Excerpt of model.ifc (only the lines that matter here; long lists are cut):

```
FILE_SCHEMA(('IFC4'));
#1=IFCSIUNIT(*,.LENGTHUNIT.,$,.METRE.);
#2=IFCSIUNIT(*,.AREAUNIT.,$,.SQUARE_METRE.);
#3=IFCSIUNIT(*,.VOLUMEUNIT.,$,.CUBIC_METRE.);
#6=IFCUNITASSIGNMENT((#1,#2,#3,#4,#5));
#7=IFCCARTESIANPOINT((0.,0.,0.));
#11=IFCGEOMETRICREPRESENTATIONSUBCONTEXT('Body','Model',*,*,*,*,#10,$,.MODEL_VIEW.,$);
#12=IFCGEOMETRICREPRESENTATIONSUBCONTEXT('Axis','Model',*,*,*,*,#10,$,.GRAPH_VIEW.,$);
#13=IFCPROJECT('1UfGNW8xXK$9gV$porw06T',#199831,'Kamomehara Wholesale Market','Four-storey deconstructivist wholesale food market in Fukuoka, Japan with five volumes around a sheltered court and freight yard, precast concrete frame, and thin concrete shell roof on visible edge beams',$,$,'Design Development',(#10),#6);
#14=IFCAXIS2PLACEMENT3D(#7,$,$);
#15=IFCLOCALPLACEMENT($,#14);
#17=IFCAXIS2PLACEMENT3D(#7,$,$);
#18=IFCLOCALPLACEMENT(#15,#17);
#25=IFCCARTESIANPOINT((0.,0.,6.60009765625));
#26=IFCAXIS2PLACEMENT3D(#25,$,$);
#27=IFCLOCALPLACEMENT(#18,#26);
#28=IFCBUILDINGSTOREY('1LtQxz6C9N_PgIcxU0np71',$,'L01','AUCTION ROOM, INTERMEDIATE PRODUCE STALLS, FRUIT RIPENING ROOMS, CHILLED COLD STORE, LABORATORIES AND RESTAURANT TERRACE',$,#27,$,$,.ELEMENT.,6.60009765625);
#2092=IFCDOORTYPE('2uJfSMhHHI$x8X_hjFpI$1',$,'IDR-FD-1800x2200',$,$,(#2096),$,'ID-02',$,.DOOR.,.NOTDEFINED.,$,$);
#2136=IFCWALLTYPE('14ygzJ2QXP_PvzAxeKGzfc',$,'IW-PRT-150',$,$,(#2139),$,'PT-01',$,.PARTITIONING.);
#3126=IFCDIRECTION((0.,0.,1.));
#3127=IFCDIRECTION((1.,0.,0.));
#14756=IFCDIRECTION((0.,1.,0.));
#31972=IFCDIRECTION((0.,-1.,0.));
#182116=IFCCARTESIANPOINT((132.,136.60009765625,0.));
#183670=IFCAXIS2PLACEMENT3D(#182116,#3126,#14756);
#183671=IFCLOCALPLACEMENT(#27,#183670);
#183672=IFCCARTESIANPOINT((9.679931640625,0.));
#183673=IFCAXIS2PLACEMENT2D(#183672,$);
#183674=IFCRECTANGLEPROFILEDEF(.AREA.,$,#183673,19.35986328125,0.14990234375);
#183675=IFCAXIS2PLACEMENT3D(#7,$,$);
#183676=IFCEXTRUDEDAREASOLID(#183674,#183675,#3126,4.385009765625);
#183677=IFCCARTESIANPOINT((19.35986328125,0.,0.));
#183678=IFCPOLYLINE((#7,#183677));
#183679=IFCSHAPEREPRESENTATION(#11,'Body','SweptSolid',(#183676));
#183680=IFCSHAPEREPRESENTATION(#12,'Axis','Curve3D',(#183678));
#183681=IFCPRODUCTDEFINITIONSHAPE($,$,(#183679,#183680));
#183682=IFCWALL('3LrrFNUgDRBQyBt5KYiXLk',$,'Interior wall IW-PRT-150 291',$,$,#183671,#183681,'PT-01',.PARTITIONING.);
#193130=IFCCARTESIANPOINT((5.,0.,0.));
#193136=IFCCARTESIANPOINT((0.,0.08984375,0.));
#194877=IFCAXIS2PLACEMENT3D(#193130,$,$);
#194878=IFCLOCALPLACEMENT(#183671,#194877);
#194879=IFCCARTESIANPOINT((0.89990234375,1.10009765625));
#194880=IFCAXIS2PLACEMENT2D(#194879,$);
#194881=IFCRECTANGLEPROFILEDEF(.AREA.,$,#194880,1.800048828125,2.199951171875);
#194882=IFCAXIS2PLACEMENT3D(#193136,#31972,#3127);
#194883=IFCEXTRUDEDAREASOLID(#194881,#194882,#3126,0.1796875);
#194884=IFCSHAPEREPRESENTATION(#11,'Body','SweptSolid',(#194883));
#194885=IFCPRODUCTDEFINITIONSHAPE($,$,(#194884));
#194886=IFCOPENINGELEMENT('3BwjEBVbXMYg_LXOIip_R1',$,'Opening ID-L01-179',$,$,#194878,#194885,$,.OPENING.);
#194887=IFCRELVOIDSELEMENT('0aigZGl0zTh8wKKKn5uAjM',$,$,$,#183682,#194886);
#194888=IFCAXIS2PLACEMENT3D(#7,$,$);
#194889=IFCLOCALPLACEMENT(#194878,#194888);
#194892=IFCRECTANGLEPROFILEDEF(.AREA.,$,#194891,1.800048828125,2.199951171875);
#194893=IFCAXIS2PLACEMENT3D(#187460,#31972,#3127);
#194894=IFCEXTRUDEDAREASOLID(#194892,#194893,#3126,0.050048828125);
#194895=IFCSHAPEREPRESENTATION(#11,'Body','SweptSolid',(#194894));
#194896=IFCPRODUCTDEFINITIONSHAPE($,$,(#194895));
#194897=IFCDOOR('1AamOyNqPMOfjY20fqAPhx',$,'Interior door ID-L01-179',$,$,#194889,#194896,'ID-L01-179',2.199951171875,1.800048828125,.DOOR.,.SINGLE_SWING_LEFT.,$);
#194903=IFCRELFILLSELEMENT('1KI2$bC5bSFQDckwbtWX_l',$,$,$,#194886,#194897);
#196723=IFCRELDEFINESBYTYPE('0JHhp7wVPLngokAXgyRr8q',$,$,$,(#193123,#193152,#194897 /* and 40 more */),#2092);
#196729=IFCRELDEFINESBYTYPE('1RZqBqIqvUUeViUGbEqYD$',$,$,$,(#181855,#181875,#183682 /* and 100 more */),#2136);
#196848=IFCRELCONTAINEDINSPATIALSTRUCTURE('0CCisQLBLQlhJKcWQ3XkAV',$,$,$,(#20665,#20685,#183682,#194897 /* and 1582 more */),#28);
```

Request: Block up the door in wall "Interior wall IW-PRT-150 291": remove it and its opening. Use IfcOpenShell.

```python
import ifcopenshell
import ifcopenshell.api.feature
import ifcopenshell.api.root
import ifcopenshell.geom
import ifcopenshell.util.shape

model = ifcopenshell.open("model.ifc")
settings = ifcopenshell.geom.settings()


def volume(element):
    """Net volume in cubic metres, openings subtracted."""
    shape = ifcopenshell.geom.create_shape(settings, element)
    return ifcopenshell.util.shape.get_volume(shape.geometry)


door = model.by_guid("1AamOyNqPMOfjY20fqAPhx")
opening = door.FillsVoids[0].RelatingOpeningElement
wall = opening.VoidsElements[0].RelatingBuildingElement
before = volume(wall)

ifcopenshell.api.root.remove_product(model, product=door)
ifcopenshell.api.feature.remove_feature(model, feature=opening)

after = volume(wall)

print(f"wall volume {before:.3f} -> {after:.3f} m3")

model.write("model-out.ifc")
```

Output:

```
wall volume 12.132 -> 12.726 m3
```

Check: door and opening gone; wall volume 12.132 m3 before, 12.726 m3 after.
